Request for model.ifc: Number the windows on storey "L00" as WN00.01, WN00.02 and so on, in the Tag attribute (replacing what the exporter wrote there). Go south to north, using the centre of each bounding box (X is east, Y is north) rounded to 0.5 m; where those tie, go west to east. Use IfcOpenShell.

First a look at what the model holds.

```python
import ifcopenshell
import ifcopenshell.util.element
import ifcopenshell.util.placement

model = ifcopenshell.open("model.ifc")
print(model.schema)
storey = next(s for s in model.by_type("IfcBuildingStorey") if s.Name == "L00")
windows = [e for e in ifcopenshell.util.element.get_decomposition(storey) if e.is_a("IfcWindow")]
for e in sorted(windows, key=lambda e: e.id()):
    origin = ifcopenshell.util.placement.get_local_placement(e.ObjectPlacement)[:3, 3]
    print(e.id(), e.Tag, e.Name, origin.round(2) + 0.0, sep=" | ")
```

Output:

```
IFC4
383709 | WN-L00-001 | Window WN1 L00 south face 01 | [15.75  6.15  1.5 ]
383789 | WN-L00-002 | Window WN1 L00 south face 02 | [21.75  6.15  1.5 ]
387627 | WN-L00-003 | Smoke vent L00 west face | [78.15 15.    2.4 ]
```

```python
import ifcopenshell
import ifcopenshell.geom
import ifcopenshell.util.element
import ifcopenshell.util.shape

model = ifcopenshell.open("model.ifc")
settings = ifcopenshell.geom.settings()
settings.set("use-world-coords", True)


def centre(element):
    shape = ifcopenshell.geom.create_shape(settings, element)
    return ifcopenshell.util.shape.get_bbox_centroid(shape.geometry)


storey = next(s for s in model.by_type("IfcBuildingStorey") if s.Name == "L00")
windows = [e for e in ifcopenshell.util.element.get_decomposition(storey) if e.is_a("IfcWindow")]

# Insertion points can sit at a corner or the storey origin, so sort by the geometry (in metres).
centres = {e: centre(e) for e in windows}
windows.sort(key=lambda e: (round(centres[e][1] / 0.5), centres[e][0]))

for i, e in enumerate(windows, start=1):
    number = f"WN00.{i:02d}"
    e.Tag = number
    print(e.id(), number)

model.write("model_rev.ifc")
```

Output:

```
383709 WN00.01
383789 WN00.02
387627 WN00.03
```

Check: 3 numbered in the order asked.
